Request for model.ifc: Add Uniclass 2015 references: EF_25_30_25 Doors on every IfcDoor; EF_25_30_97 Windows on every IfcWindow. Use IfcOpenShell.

First a look at what the model holds.

```python
import ifcopenshell

model = ifcopenshell.open("model.ifc")
print(model.schema)
print("classifications:", [c.Name for c in model.by_type("IfcClassification")])
for ifc_class in ("IfcDoor", "IfcRoof", "IfcStair", "IfcWall", "IfcWindow"):
    print(ifc_class, len(model.by_type(ifc_class)))
```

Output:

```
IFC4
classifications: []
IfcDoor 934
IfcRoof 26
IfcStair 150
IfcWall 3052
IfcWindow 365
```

```python
import ifcopenshell
import ifcopenshell.api.classification

model = ifcopenshell.open("model.ifc")

system = ifcopenshell.api.classification.add_classification(model, classification="Uniclass 2015")

codes = {
    "IfcDoor": ("EF_25_30_25", "Doors"),
    "IfcWindow": ("EF_25_30_97", "Windows"),
}
for ifc_class, (code, name) in codes.items():
    products = model.by_type(ifc_class)
    ifcopenshell.api.classification.add_reference(
        model, products=products, classification=system, identification=code, name=name
    )
    print(code, len(products))

model.write("model_v2.ifc")
```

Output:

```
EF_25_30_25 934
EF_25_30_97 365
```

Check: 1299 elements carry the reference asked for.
